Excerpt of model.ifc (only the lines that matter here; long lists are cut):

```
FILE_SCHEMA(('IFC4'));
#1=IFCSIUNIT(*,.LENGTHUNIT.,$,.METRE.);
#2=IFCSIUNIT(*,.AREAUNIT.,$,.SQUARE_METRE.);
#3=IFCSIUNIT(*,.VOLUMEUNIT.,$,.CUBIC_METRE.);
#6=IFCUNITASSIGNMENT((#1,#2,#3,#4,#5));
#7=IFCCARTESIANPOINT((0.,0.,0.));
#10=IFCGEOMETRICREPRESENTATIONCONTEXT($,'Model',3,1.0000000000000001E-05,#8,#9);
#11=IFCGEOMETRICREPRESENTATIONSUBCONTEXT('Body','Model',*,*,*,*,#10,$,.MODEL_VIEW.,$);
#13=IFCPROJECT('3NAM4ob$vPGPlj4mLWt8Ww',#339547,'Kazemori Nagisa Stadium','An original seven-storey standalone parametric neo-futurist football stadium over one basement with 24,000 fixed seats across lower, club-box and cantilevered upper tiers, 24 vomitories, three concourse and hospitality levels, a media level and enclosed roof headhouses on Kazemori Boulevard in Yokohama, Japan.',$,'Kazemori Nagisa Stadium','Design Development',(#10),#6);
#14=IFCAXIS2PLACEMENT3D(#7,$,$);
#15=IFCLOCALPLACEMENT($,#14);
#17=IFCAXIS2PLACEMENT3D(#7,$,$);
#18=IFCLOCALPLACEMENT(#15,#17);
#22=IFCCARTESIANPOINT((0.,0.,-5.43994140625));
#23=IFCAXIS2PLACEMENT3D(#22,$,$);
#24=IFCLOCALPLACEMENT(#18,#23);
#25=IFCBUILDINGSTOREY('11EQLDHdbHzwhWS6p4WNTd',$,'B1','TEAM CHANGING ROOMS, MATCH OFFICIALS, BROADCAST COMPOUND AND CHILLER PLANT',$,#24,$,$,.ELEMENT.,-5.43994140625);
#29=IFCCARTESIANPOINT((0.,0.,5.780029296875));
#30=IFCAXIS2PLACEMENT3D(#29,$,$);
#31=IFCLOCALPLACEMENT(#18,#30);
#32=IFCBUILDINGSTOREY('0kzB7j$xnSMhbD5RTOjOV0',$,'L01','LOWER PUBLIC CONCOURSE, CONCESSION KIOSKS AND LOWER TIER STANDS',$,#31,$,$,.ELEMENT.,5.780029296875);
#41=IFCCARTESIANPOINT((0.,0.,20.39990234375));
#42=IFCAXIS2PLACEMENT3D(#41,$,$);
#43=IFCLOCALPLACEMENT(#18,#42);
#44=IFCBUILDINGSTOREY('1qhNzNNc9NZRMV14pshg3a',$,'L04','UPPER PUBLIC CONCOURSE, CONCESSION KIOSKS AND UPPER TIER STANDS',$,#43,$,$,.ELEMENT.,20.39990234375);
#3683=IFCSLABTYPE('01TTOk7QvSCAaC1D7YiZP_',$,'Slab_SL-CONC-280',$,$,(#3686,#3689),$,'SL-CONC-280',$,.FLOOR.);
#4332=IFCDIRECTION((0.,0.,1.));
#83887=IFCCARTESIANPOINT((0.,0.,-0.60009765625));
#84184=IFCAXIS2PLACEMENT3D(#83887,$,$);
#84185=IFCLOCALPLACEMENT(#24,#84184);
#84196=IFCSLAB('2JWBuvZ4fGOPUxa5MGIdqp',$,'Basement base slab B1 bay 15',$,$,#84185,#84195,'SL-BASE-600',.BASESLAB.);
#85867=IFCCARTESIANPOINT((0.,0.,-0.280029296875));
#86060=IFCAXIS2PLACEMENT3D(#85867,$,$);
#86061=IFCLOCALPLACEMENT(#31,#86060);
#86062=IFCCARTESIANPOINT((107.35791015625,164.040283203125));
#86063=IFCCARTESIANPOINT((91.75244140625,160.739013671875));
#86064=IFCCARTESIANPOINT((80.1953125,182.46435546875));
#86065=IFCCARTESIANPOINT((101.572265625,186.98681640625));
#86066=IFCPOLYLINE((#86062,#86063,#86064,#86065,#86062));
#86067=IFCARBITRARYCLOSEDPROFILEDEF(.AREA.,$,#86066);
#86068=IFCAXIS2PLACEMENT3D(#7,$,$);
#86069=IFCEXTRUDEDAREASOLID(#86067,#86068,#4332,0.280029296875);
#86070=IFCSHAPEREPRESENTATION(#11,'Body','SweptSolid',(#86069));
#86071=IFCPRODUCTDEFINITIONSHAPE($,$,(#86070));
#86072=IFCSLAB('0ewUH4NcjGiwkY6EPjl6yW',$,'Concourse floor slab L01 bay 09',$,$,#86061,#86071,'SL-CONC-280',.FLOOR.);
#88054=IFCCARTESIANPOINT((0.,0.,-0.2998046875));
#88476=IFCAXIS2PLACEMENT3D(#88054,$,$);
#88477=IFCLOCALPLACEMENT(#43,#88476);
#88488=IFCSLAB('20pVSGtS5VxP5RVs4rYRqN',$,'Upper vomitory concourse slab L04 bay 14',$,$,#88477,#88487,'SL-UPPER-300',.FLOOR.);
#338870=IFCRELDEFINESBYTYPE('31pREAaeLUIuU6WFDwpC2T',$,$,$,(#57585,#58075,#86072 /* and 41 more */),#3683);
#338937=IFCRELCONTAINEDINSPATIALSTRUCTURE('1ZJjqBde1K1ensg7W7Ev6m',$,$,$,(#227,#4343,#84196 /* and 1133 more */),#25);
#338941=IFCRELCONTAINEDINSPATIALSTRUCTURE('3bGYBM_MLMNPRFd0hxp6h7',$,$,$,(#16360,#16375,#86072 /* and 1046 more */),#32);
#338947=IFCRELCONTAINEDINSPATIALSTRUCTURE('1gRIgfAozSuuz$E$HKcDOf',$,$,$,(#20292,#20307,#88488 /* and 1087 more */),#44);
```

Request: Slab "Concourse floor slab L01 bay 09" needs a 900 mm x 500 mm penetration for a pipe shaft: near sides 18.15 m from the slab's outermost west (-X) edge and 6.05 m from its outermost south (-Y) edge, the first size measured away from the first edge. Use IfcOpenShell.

```python
import numpy as np
import ifcopenshell
import ifcopenshell.api.feature
import ifcopenshell.api.geometry
import ifcopenshell.api.root
import ifcopenshell.geom
import ifcopenshell.util.placement
import ifcopenshell.util.representation
import ifcopenshell.util.shape
import ifcopenshell.util.unit

model = ifcopenshell.open("model.ifc")
unit_scale = ifcopenshell.util.unit.calculate_unit_scale(model)
settings = ifcopenshell.geom.settings()


def volume(element):
    """Net volume in cubic metres, openings subtracted."""
    shape = ifcopenshell.geom.create_shape(settings, element)
    return ifcopenshell.util.shape.get_volume(shape.geometry)


slab = model.by_guid("0ewUH4NcjGiwkY6EPjl6yW")
before = volume(slab)

# Extent in the slab's own axes, in metres. The edges named are its -X and -Y sides.
slab_shape = ifcopenshell.geom.create_shape(settings, slab)
vertices = ifcopenshell.util.shape.get_vertices(slab_shape.geometry)
x_min, y_min, bottom = vertices.min(axis=0)
top = vertices[:, 2].max()

opening = ifcopenshell.api.root.create_entity(model, ifc_class="IfcOpeningElement", name="Pipe shaft opening", predefined_type="OPENING")
context = ifcopenshell.util.representation.get_context(model, "Model", "Body", "MODEL_VIEW")
width, depth = 0.9, 0.5
outline = [(0.0, 0.0), (width, 0.0), (width, depth), (0.0, depth), (0.0, 0.0)]
# Overshoot both faces by 50 mm so the cut is clean.
shape = ifcopenshell.api.geometry.add_slab_representation(
    model, context=context, depth=top - bottom + 0.1, polyline=outline
)
ifcopenshell.api.geometry.assign_representation(model, product=opening, representation=shape)

matrix = ifcopenshell.util.placement.get_local_placement(slab.ObjectPlacement)
matrix[:, 3] = matrix @ np.append(np.array([x_min + 18.15, y_min + 6.05, bottom - 0.05]) / unit_scale, 1.0)
ifcopenshell.api.geometry.edit_object_placement(model, product=opening, matrix=matrix, is_si=False)
ifcopenshell.api.feature.add_feature(model, feature=opening, element=slab)

after = volume(slab)

print(f"slab volume {before:.3f} -> {after:.3f} m3")

model.write("model_edited.ifc")
```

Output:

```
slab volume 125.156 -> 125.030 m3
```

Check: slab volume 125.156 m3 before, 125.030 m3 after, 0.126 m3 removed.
